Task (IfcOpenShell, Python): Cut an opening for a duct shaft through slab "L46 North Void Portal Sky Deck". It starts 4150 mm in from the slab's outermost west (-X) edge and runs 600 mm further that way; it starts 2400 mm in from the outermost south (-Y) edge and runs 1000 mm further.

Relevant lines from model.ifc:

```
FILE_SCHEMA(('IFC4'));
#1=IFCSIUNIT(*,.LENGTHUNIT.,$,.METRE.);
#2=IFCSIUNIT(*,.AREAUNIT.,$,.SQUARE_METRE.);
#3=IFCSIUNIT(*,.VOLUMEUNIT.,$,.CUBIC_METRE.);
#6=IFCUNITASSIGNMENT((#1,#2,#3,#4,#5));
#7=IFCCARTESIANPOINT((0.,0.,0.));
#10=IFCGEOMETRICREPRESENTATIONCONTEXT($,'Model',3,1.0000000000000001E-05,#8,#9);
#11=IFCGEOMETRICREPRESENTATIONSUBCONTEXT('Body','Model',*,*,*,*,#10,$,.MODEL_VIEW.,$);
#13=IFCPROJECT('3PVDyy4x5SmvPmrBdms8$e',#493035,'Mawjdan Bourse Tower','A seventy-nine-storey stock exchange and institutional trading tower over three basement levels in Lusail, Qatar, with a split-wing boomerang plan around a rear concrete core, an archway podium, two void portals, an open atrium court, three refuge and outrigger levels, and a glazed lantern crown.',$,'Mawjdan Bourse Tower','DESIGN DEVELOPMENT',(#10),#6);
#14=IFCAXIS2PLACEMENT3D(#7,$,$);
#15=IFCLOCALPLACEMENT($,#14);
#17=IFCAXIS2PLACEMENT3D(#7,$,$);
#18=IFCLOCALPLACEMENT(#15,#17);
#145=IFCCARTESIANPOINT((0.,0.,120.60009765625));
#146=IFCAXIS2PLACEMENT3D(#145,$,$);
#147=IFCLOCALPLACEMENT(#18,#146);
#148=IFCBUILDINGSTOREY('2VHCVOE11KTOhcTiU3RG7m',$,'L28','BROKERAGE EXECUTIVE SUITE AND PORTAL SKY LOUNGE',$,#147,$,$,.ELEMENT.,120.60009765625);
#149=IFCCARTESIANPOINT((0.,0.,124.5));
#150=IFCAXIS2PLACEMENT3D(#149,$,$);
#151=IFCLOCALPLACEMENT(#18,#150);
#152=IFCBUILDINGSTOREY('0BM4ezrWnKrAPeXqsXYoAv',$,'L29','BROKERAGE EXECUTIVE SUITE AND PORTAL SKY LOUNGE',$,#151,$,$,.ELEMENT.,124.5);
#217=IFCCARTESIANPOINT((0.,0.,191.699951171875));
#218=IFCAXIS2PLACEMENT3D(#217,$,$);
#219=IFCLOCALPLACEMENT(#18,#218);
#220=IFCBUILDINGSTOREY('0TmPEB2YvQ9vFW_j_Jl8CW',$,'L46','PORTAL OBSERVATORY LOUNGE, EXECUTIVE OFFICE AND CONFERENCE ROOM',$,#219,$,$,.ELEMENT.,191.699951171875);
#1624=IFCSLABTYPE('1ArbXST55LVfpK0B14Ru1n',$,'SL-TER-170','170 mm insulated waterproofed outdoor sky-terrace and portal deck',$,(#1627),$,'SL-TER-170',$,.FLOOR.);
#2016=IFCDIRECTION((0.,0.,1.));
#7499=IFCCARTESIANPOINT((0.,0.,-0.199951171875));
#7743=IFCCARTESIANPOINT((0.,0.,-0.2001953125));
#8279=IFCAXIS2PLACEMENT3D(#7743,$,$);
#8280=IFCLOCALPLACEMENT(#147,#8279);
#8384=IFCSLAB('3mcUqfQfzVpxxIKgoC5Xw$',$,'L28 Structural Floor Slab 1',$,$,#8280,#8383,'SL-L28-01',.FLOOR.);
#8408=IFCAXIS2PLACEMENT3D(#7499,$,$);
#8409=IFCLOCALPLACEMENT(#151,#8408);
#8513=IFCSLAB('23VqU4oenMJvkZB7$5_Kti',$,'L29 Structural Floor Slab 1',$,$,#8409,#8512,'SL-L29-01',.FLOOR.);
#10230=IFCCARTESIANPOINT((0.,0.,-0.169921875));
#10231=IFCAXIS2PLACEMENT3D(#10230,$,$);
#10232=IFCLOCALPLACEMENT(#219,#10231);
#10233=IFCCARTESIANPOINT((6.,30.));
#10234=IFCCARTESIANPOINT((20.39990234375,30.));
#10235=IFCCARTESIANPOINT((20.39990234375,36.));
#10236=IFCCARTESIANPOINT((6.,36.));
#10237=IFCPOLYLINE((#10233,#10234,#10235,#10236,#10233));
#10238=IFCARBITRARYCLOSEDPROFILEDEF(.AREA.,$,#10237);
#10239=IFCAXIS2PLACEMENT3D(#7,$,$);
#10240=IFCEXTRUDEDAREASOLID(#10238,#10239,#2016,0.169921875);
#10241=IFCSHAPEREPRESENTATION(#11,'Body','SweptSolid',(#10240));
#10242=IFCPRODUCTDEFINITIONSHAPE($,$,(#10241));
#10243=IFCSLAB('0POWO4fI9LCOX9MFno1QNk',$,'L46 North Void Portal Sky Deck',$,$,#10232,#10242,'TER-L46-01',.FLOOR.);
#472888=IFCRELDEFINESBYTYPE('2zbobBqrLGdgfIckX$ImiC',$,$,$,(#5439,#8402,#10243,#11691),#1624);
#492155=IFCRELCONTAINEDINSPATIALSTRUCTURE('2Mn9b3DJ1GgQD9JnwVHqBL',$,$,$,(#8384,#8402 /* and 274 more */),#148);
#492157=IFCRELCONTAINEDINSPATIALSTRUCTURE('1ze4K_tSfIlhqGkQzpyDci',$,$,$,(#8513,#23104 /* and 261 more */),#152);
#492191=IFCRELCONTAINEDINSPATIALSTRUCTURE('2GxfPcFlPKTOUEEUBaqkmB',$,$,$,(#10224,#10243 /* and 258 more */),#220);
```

```python
import numpy as np
import ifcopenshell
import ifcopenshell.api.feature
import ifcopenshell.api.geometry
import ifcopenshell.api.root
import ifcopenshell.geom
import ifcopenshell.util.placement
import ifcopenshell.util.representation
import ifcopenshell.util.shape
import ifcopenshell.util.unit

model = ifcopenshell.open("model.ifc")
unit_scale = ifcopenshell.util.unit.calculate_unit_scale(model)
settings = ifcopenshell.geom.settings()


def volume(element):
    """Net volume in cubic metres, openings subtracted."""
    shape = ifcopenshell.geom.create_shape(settings, element)
    return ifcopenshell.util.shape.get_volume(shape.geometry)


slab = model.by_guid("0POWO4fI9LCOX9MFno1QNk")
before = volume(slab)

# Extent in the slab's own axes, in metres. The edges named are its -X and -Y sides.
slab_shape = ifcopenshell.geom.create_shape(settings, slab)
vertices = ifcopenshell.util.shape.get_vertices(slab_shape.geometry)
x_min, y_min, bottom = vertices.min(axis=0)
top = vertices[:, 2].max()

opening = ifcopenshell.api.root.create_entity(model, ifc_class="IfcOpeningElement", name="Duct shaft opening", predefined_type="OPENING")
context = ifcopenshell.util.representation.get_context(model, "Model", "Body", "MODEL_VIEW")
width, depth = 0.6, 1
outline = [(0.0, 0.0), (width, 0.0), (width, depth), (0.0, depth), (0.0, 0.0)]
# Overshoot both faces by 50 mm so the cut is clean.
shape = ifcopenshell.api.geometry.add_slab_representation(
    model, context=context, depth=top - bottom + 0.1, polyline=outline
)
ifcopenshell.api.geometry.assign_representation(model, product=opening, representation=shape)

matrix = ifcopenshell.util.placement.get_local_placement(slab.ObjectPlacement)
matrix[:, 3] = matrix @ np.append(np.array([x_min + 4.15, y_min + 2.4, bottom - 0.05]) / unit_scale, 1.0)
ifcopenshell.api.geometry.edit_object_placement(model, product=opening, matrix=matrix, is_si=False)
ifcopenshell.api.feature.add_feature(model, feature=opening, element=slab)

after = volume(slab)

print(f"slab volume {before:.3f} -> {after:.3f} m3")

model.write("model_rev.ifc")
```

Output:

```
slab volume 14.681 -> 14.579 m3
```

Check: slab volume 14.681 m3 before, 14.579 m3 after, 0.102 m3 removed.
